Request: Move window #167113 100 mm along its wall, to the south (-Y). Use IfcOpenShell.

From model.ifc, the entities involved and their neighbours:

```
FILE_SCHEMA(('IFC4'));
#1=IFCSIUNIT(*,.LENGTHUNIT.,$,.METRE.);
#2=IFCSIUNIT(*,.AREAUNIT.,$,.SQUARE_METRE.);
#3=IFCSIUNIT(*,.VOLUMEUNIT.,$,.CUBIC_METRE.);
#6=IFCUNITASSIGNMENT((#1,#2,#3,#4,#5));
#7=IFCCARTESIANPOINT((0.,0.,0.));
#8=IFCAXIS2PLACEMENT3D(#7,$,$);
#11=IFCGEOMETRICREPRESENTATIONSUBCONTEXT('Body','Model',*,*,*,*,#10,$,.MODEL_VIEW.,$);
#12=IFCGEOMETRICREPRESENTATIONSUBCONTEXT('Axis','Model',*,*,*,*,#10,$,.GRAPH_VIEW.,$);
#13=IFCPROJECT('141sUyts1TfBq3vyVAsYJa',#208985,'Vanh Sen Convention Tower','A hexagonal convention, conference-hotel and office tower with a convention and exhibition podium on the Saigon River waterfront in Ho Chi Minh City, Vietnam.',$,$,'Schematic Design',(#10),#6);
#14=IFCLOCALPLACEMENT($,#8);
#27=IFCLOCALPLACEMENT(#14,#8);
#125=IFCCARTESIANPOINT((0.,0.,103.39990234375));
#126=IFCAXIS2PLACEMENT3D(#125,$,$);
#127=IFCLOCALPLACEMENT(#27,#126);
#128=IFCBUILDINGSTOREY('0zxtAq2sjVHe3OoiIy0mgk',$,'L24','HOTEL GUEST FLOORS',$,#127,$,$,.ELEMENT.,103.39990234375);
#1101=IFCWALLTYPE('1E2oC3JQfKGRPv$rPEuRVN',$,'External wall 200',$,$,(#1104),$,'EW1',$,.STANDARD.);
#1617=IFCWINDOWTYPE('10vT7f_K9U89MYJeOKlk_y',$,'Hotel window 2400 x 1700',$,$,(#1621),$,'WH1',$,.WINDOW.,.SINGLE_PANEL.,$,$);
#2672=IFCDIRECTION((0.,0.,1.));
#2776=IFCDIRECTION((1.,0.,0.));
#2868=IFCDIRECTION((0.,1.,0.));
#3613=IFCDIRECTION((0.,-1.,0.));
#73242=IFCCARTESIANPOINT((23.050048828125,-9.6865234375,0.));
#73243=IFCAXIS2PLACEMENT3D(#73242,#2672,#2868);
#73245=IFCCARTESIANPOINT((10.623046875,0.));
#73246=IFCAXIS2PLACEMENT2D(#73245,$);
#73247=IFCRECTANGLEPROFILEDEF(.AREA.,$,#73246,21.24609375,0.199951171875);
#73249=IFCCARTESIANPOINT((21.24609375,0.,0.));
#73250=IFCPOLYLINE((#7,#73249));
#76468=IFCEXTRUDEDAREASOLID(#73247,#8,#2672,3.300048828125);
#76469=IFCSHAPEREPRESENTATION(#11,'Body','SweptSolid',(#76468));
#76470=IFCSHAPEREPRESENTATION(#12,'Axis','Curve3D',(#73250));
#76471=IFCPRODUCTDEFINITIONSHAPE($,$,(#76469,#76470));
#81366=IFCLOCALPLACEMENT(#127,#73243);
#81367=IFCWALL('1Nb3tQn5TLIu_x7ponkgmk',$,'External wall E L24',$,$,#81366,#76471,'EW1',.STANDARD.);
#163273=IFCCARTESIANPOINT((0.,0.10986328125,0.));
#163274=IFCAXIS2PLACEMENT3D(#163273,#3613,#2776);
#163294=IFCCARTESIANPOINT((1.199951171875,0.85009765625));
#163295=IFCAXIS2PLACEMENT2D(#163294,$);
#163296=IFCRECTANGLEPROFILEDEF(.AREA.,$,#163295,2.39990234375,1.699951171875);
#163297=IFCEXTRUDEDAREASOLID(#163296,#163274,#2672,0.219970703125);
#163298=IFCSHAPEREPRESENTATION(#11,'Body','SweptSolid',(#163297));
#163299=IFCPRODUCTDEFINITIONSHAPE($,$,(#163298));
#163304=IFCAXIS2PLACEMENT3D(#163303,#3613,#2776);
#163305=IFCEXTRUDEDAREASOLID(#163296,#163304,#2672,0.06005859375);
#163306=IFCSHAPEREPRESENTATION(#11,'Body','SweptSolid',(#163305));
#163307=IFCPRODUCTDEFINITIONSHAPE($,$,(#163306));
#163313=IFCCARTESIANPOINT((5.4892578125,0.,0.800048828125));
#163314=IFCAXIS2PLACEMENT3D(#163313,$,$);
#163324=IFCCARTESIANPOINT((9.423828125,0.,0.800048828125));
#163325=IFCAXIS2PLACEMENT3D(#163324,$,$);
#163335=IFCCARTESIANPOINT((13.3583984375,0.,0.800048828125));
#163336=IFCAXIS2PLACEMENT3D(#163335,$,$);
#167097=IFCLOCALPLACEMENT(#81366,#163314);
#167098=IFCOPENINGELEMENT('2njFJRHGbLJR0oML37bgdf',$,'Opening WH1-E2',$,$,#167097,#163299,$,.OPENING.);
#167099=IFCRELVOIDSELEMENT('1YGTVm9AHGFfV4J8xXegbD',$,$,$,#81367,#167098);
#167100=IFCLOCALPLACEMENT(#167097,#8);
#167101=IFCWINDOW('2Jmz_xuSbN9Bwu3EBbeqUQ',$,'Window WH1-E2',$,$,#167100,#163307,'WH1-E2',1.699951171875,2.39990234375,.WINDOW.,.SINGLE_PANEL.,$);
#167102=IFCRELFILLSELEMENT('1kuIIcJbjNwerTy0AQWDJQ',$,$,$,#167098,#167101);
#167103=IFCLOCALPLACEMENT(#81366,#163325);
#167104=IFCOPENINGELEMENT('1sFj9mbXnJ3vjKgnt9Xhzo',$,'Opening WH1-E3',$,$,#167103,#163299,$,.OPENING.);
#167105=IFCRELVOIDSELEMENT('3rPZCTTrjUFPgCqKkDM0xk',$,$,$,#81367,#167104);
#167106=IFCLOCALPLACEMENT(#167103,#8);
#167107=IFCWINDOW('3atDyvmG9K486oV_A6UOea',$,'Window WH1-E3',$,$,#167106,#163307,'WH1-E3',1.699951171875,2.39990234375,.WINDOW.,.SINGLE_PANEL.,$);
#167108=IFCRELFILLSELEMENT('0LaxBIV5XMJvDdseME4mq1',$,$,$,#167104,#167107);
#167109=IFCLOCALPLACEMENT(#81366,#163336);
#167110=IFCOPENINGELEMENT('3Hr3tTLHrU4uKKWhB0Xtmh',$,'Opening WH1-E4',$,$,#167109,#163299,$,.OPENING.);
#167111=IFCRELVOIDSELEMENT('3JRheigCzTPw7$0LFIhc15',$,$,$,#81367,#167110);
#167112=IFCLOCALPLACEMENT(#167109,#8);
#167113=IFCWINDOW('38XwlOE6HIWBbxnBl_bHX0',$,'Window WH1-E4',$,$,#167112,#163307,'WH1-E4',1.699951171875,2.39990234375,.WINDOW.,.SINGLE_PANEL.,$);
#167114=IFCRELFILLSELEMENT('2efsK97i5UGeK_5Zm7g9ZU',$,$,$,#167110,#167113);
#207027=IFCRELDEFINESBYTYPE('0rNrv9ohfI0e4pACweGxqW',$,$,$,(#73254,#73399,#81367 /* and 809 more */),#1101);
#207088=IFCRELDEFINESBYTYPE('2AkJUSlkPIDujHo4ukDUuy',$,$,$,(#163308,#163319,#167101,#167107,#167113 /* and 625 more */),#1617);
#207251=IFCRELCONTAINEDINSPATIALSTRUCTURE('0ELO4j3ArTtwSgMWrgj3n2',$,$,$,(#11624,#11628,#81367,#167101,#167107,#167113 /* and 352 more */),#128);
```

```python
import ifcopenshell
import ifcopenshell.api.geometry
import ifcopenshell.util.placement

model = ifcopenshell.open("model.ifc")

window = model.by_id(167113)
opening = window.FillsVoids[0].RelatingOpeningElement
wall = opening.VoidsElements[0].RelatingBuildingElement

wall_matrix = ifcopenshell.util.placement.get_local_placement(wall.ObjectPlacement)
shift = wall_matrix[:3, 0] * -0.1
before = ifcopenshell.util.placement.get_local_placement(window.ObjectPlacement)[:3, 3].copy()

# The window is placed relative to its opening, so it follows when the opening moves.
matrix = ifcopenshell.util.placement.get_local_placement(opening.ObjectPlacement)
matrix[:3, 3] += shift
ifcopenshell.api.geometry.edit_object_placement(
    model, product=opening, matrix=matrix, is_si=False, should_transform_children=True
)

after = ifcopenshell.util.placement.get_local_placement(window.ObjectPlacement)[:3, 3]
print("window moved by", (after - before).round(3) + 0.0)

model.write("model_edited.ifc")
```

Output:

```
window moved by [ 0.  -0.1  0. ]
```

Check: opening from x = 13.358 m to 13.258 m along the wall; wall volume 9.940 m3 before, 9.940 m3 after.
